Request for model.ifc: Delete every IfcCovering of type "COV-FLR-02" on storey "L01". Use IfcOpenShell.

First a look at what the model holds.

```python
import ifcopenshell
import ifcopenshell.util.element

model = ifcopenshell.open("model.ifc")
print(model.schema)
storey = next(s for s in model.by_type("IfcBuildingStorey") if s.Name == "L01")
coverings = [e for e in ifcopenshell.util.element.get_decomposition(storey) if e.is_a("IfcCovering")]
seen = {}
for e in coverings:
    element_type = ifcopenshell.util.element.get_type(e)
    name = element_type.Name if element_type not in (None, e) else None
    seen[name] = seen.get(name, 0) + 1
for name, count in sorted(seen.items(), key=str):
    print(count, "x", name)
```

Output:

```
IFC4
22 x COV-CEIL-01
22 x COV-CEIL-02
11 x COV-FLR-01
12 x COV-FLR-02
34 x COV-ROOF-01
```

```python
import ifcopenshell
import ifcopenshell.api.root
import ifcopenshell.util.element

model = ifcopenshell.open("model.ifc")

storey = next(s for s in model.by_type("IfcBuildingStorey") if s.Name == "L01")
coverings = [e for e in ifcopenshell.util.element.get_decomposition(storey) if e.is_a("IfcCovering")]
targets = [e for e in coverings if (t := ifcopenshell.util.element.get_type(e)) not in (None, e) and t.Name == "COV-FLR-02"]

for e in targets:
    ifcopenshell.api.root.remove_product(model, product=e)
print(len(targets), "removed")

model.write("model_rev.ifc")
```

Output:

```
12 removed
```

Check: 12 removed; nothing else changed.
